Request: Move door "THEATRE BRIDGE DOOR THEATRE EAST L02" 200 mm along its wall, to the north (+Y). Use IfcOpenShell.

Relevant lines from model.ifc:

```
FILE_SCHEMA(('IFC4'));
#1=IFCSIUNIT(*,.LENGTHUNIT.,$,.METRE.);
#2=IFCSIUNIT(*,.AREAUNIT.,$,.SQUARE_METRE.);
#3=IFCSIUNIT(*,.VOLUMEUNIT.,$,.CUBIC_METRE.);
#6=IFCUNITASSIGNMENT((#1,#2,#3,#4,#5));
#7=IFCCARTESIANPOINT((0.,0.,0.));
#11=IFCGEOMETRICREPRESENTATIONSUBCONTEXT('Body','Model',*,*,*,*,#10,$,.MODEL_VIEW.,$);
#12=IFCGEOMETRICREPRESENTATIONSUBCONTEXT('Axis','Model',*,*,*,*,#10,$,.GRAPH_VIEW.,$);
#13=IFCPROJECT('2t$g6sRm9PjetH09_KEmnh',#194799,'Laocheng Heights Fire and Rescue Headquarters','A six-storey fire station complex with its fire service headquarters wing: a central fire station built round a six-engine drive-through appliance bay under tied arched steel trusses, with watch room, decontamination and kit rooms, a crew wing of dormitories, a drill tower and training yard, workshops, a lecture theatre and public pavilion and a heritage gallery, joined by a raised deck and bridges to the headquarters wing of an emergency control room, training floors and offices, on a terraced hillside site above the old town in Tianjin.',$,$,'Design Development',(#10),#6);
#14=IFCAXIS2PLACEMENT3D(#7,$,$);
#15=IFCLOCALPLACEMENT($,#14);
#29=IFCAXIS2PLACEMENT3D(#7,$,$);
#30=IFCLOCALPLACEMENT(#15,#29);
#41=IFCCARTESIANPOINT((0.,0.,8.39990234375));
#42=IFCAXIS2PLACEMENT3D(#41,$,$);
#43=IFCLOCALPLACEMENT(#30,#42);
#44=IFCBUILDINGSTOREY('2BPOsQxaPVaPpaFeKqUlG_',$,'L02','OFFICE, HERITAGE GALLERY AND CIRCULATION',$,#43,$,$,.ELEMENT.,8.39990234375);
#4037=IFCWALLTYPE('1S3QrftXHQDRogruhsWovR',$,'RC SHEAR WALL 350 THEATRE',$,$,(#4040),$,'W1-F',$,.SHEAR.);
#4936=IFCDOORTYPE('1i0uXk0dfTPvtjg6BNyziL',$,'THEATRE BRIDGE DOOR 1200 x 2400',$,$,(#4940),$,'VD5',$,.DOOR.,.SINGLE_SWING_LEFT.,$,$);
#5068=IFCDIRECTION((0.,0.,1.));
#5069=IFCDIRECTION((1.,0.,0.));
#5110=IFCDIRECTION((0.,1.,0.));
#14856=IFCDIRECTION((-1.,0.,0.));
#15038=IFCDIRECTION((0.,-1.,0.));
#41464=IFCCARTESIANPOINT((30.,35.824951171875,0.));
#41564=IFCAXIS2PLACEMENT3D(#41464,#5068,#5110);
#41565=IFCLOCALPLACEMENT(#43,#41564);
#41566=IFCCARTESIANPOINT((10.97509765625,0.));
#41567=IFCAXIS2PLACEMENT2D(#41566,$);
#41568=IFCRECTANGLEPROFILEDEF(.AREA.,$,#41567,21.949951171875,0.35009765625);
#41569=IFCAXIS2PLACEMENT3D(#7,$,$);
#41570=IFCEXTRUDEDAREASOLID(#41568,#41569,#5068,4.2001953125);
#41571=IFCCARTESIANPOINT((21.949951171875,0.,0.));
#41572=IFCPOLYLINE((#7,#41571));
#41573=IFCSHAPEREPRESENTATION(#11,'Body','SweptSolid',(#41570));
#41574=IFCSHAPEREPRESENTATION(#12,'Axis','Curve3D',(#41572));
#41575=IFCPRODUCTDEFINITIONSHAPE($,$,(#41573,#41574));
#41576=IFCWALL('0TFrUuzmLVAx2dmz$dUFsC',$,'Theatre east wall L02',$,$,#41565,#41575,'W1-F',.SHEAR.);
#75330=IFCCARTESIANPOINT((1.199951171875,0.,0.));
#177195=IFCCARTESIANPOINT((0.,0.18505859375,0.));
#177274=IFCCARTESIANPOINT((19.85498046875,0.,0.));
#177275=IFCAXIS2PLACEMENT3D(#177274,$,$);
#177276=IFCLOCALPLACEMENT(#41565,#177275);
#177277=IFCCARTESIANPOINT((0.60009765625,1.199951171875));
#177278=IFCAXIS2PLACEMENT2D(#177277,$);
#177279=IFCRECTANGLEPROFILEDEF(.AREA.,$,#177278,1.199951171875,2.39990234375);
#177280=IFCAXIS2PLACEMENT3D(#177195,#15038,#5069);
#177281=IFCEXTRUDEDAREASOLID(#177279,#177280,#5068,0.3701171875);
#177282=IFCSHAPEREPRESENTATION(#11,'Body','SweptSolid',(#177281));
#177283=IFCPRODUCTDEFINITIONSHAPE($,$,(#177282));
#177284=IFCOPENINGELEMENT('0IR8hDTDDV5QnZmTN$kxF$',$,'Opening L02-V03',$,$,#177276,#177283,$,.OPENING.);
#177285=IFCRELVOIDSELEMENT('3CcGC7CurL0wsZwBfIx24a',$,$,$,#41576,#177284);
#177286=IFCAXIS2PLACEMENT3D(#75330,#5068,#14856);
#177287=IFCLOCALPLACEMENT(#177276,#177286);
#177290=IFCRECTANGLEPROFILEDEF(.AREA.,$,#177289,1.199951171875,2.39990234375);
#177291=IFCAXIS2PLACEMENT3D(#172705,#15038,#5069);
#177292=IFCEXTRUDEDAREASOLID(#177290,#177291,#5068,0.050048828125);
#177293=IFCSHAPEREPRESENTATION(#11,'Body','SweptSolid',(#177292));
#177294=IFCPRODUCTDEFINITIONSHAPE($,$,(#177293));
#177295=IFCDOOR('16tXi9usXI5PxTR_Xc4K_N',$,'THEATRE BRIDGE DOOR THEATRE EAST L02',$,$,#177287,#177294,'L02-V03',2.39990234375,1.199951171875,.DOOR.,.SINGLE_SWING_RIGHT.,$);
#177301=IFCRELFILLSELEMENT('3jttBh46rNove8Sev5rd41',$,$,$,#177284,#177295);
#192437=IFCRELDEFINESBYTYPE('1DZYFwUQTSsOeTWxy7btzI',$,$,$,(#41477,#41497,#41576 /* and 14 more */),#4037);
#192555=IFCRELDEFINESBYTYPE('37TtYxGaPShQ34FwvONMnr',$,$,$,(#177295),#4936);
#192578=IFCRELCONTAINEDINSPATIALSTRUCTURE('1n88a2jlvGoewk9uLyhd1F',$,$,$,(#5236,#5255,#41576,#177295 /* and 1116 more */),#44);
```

```python
import ifcopenshell
import ifcopenshell.api.geometry
import ifcopenshell.util.placement

model = ifcopenshell.open("model.ifc")

door = model.by_id(177295)
opening = door.FillsVoids[0].RelatingOpeningElement
wall = opening.VoidsElements[0].RelatingBuildingElement

wall_matrix = ifcopenshell.util.placement.get_local_placement(wall.ObjectPlacement)
shift = wall_matrix[:3, 0] * 0.2
before = ifcopenshell.util.placement.get_local_placement(door.ObjectPlacement)[:3, 3].copy()

# The door is placed relative to its opening, so it follows when the opening moves.
matrix = ifcopenshell.util.placement.get_local_placement(opening.ObjectPlacement)
matrix[:3, 3] += shift
ifcopenshell.api.geometry.edit_object_placement(
    model, product=opening, matrix=matrix, is_si=False, should_transform_children=True
)

after = ifcopenshell.util.placement.get_local_placement(door.ObjectPlacement)[:3, 3]
print("door moved by", (after - before).round(3) + 0.0)

model.write("model_rev.ifc")
```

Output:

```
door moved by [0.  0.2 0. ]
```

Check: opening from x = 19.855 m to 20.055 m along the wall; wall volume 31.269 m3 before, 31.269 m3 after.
